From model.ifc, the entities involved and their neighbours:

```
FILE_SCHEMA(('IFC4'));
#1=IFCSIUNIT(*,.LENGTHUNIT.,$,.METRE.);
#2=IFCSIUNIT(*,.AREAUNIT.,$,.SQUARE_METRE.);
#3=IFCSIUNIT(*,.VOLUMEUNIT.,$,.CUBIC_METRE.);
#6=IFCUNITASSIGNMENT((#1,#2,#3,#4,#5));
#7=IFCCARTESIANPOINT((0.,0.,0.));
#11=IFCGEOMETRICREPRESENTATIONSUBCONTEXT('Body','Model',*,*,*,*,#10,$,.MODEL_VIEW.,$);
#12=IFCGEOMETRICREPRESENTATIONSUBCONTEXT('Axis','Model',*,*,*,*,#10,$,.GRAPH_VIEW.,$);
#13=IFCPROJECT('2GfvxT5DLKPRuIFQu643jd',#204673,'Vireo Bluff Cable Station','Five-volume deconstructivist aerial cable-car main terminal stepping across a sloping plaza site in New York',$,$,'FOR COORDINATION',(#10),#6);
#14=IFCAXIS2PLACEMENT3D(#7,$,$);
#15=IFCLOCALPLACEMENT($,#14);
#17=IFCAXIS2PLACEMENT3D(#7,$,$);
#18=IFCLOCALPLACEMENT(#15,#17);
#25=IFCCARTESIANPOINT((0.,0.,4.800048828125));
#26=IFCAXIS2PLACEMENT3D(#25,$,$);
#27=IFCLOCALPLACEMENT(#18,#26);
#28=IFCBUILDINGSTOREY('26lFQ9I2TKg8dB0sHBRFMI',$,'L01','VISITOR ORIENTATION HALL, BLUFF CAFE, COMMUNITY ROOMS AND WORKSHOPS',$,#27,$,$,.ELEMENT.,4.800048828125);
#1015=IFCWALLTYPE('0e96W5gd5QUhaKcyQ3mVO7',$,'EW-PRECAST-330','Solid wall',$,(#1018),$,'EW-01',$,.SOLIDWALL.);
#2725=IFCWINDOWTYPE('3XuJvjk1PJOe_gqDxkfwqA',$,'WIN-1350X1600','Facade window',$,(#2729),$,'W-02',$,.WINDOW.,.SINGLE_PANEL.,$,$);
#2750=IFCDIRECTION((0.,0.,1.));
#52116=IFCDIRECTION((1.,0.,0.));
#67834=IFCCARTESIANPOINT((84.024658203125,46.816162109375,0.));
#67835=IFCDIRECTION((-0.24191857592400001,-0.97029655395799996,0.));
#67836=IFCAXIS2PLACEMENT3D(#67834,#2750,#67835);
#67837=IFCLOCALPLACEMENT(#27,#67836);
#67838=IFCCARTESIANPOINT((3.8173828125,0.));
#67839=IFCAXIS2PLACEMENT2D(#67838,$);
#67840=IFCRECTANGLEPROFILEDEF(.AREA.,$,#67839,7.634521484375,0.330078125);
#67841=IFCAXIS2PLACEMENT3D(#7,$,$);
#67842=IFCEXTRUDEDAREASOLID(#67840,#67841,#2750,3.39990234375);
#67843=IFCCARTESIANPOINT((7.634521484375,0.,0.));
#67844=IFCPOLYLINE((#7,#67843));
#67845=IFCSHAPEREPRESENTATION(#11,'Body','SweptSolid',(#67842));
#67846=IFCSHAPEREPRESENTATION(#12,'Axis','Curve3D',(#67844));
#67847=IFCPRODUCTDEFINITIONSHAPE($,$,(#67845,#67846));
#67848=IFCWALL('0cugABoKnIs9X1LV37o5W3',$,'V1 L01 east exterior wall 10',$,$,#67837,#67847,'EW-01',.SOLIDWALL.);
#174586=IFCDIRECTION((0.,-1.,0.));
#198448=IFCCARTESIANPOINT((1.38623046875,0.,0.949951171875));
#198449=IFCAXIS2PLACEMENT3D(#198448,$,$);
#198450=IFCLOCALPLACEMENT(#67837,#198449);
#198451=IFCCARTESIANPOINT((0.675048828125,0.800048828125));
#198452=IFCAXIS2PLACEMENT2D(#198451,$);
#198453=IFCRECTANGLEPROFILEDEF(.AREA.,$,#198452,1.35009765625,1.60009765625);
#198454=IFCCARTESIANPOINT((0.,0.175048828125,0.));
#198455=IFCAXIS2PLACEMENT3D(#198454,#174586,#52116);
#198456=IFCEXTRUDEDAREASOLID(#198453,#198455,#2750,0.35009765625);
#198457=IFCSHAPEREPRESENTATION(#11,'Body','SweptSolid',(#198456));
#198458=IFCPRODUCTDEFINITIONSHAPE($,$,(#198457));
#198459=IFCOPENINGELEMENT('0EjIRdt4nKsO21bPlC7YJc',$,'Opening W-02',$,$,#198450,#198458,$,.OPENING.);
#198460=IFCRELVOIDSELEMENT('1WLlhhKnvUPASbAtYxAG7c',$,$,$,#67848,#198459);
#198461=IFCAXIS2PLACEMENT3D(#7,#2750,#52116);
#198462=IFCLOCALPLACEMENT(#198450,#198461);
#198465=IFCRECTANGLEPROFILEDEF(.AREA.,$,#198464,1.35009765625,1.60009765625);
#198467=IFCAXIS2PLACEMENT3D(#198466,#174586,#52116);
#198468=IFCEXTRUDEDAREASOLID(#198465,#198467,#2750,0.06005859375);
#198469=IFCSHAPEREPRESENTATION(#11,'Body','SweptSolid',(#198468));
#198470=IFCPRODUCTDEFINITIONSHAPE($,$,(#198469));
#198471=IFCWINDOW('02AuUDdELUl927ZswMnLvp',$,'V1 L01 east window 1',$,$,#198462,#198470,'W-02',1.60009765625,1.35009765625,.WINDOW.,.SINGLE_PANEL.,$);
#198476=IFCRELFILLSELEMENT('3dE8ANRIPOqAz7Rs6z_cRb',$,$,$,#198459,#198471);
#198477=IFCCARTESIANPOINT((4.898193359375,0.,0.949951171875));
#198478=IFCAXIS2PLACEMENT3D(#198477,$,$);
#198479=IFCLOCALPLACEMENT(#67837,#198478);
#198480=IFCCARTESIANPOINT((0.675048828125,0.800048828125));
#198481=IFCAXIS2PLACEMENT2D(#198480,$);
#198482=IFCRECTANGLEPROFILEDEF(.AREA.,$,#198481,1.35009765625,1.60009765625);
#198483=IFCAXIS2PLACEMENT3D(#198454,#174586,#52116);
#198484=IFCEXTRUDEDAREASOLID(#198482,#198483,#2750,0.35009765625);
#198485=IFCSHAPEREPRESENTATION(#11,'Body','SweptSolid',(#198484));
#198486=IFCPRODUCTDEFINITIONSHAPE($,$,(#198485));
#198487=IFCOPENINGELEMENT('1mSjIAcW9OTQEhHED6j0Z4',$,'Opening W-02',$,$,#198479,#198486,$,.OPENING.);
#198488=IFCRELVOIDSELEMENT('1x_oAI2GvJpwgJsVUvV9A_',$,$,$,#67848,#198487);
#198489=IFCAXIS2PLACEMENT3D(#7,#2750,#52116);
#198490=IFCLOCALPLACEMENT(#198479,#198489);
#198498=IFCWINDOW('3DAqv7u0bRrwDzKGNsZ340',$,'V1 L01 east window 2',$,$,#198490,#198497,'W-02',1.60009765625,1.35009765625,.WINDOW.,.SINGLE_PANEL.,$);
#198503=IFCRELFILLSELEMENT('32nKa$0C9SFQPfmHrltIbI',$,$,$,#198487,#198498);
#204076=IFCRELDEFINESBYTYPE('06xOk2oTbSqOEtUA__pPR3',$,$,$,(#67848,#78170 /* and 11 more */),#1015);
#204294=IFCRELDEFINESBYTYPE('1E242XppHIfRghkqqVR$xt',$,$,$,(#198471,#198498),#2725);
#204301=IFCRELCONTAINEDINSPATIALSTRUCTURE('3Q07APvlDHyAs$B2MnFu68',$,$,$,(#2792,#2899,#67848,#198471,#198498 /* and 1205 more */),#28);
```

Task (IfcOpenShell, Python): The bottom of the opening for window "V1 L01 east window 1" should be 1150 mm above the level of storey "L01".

```python
import numpy as np
import ifcopenshell
import ifcopenshell.api.geometry
import ifcopenshell.geom
import ifcopenshell.util.element
import ifcopenshell.util.placement
import ifcopenshell.util.shape
import ifcopenshell.util.unit

model = ifcopenshell.open("model.ifc")
unit_scale = ifcopenshell.util.unit.calculate_unit_scale(model)

window = model.by_guid("02AuUDdELUl927ZswMnLvp")
opening = window.FillsVoids[0].RelatingOpeningElement
storey = ifcopenshell.util.element.get_container(window, ifc_class="IfcBuildingStorey")
level = ifcopenshell.util.placement.get_local_placement(storey.ObjectPlacement)[2, 3]

# The opening's origin need not be at the sill, so measure its lowest point.
shape = ifcopenshell.geom.create_shape(ifcopenshell.geom.settings(), opening)
bottom = ifcopenshell.util.shape.get_shape_bottom_elevation(shape, shape.geometry) / unit_scale
dz = level + 1.15 / unit_scale - bottom

shift = np.array([0.0, 0.0, dz])
# The window is placed relative to its opening, so it follows when the opening moves.
matrix = ifcopenshell.util.placement.get_local_placement(opening.ObjectPlacement)
matrix[:3, 3] += shift
ifcopenshell.api.geometry.edit_object_placement(
    model, product=opening, matrix=matrix, is_si=False, should_transform_children=True
)

print(f"moved by {dz * unit_scale:+.3f} m")

model.write("model_rev.ifc")
```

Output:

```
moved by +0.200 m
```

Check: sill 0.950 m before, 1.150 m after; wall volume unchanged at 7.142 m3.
